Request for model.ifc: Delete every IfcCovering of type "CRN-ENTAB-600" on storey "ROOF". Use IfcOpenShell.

First a look at what the model holds.

```python
import ifcopenshell
import ifcopenshell.util.element

model = ifcopenshell.open("model.ifc")
print(model.schema)
storey = next(s for s in model.by_type("IfcBuildingStorey") if s.Name == "ROOF")
coverings = [e for e in ifcopenshell.util.element.get_decomposition(storey) if e.is_a("IfcCovering")]
seen = {}
for e in coverings:
    element_type = ifcopenshell.util.element.get_type(e)
    name = element_type.Name if element_type not in (None, e) else None
    seen[name] = seen.get(name, 0) + 1
for name, count in sorted(seen.items(), key=str):
    print(count, "x", name)
```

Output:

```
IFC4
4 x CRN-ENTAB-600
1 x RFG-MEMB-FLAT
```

```python
import ifcopenshell
import ifcopenshell.api.root
import ifcopenshell.util.element

model = ifcopenshell.open("model.ifc")

storey = next(s for s in model.by_type("IfcBuildingStorey") if s.Name == "ROOF")
coverings = [e for e in ifcopenshell.util.element.get_decomposition(storey) if e.is_a("IfcCovering")]
targets = [e for e in coverings if (t := ifcopenshell.util.element.get_type(e)) not in (None, e) and t.Name == "CRN-ENTAB-600"]

for e in targets:
    ifcopenshell.api.root.remove_product(model, product=e)
print(len(targets), "removed")

model.write("model_edited.ifc")
```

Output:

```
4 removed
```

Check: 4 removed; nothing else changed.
